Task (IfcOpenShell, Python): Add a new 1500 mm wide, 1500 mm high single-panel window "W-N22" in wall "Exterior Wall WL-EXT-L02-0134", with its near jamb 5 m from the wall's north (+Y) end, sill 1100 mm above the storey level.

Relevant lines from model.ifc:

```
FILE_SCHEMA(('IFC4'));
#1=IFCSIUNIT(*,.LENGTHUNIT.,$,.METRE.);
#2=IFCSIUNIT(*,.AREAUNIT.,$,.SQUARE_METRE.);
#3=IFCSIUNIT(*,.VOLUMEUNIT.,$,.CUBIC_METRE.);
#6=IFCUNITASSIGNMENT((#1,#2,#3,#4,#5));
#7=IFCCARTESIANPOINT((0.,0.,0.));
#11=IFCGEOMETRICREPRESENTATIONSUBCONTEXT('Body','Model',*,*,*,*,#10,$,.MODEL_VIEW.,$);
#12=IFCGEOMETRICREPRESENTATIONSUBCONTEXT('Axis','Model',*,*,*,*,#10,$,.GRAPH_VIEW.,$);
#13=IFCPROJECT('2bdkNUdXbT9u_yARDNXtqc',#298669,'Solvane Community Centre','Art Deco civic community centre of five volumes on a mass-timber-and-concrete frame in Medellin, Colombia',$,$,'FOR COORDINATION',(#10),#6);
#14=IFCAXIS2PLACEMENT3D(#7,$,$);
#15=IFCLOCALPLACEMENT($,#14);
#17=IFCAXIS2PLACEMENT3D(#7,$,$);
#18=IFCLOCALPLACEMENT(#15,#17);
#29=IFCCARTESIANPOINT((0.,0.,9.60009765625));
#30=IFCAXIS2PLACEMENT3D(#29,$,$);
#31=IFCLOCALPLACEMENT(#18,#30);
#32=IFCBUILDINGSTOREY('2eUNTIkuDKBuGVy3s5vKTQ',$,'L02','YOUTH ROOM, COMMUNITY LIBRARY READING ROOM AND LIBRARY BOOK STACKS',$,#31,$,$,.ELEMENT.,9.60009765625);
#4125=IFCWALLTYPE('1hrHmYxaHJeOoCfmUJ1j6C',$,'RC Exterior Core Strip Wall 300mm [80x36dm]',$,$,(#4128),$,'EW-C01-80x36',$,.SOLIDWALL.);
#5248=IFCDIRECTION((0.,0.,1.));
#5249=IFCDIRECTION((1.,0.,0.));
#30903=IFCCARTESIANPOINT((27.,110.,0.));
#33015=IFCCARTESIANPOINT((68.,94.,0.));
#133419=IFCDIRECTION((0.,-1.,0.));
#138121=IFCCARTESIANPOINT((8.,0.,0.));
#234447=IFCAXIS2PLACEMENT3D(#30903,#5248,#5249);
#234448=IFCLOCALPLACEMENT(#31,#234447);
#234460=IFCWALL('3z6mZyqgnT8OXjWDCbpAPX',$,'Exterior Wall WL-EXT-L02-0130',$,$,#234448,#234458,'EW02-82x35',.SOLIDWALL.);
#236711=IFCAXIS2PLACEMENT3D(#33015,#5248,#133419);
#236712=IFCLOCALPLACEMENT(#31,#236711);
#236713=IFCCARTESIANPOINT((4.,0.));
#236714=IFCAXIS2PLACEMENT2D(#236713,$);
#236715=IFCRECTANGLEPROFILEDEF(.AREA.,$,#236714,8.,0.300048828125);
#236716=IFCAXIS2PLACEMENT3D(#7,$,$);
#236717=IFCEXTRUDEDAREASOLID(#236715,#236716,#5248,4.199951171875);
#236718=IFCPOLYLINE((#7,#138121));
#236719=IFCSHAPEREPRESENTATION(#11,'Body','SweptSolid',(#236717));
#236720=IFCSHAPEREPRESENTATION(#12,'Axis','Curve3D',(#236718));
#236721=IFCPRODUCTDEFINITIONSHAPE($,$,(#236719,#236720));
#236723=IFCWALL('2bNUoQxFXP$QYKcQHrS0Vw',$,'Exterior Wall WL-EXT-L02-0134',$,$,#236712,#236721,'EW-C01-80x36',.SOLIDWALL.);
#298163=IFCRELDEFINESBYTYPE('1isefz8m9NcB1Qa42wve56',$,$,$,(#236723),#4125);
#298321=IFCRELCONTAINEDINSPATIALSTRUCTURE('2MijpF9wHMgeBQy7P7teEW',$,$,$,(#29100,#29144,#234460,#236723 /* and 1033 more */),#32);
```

```python
import numpy as np
import ifcopenshell
import ifcopenshell.api.feature
import ifcopenshell.api.geometry
import ifcopenshell.api.root
import ifcopenshell.api.spatial
import ifcopenshell.geom
import ifcopenshell.util.element
import ifcopenshell.util.placement
import ifcopenshell.util.representation
import ifcopenshell.util.shape
import ifcopenshell.util.unit

model = ifcopenshell.open("model.ifc")
unit_scale = ifcopenshell.util.unit.calculate_unit_scale(model)
settings = ifcopenshell.geom.settings()


def volume(element):
    """Net volume in cubic metres, openings subtracted."""
    shape = ifcopenshell.geom.create_shape(settings, element)
    return ifcopenshell.util.shape.get_volume(shape.geometry)


wall = model.by_guid("2bNUoQxFXP$QYKcQHrS0Vw")
storey = ifcopenshell.util.element.get_container(wall, ifc_class="IfcBuildingStorey")
context = ifcopenshell.util.representation.get_context(model, "Model", "Body", "MODEL_VIEW")
before = volume(wall)

width, height, from_end, sill = 1.5, 1.5, 5, 1.1  # metres

# The wall runs along its own X axis, and the end named is its -X end.
wall_shape = ifcopenshell.geom.create_shape(settings, wall)
x, y, z = ifcopenshell.util.shape.get_vertices(wall_shape.geometry).T
start = x.min() + from_end
face, thickness = float(y.min()), float(y.max() - y.min())
wall_matrix = ifcopenshell.util.placement.get_local_placement(wall.ObjectPlacement)
level = ifcopenshell.util.placement.get_local_placement(storey.ObjectPlacement)[2, 3]


def in_wall(x, y):
    """Placement at x, y metres in the wall's axes, at sill height."""
    matrix = wall_matrix.copy()
    matrix[:, 3] = wall_matrix @ np.array([x / unit_scale, y / unit_scale, 0.0, 1.0])
    matrix[2, 3] = level + sill / unit_scale
    return matrix


# Opening: a box that overshoots both wall faces by 50 mm.
opening = ifcopenshell.api.root.create_entity(model, ifc_class="IfcOpeningElement", predefined_type="OPENING")
box = ifcopenshell.api.geometry.add_wall_representation(
    model, context=context, length=width, height=height, thickness=thickness + 0.1
)
ifcopenshell.api.geometry.assign_representation(model, product=opening, representation=box)
ifcopenshell.api.geometry.edit_object_placement(model, product=opening, matrix=in_wall(start, face - 0.05), is_si=False)
ifcopenshell.api.feature.add_feature(model, feature=opening, element=wall)

window = ifcopenshell.api.root.create_entity(model, ifc_class="IfcWindow", name="W-N22", predefined_type="WINDOW")
window.OverallWidth, window.OverallHeight = width / unit_scale, height / unit_scale
window.PartitioningType = "SINGLE_PANEL"
body = ifcopenshell.api.geometry.add_window_representation(
    model,
    context=context,
    overall_width=window.OverallWidth,
    overall_height=window.OverallHeight,
    partition_type="SINGLE_PANEL",
)
ifcopenshell.api.geometry.assign_representation(model, product=window, representation=body)
ifcopenshell.api.spatial.assign_container(model, products=[window], relating_structure=storey)
ifcopenshell.api.feature.add_filling(model, opening=opening, element=window)

# Centre the window in the wall's thickness.
ifcopenshell.api.geometry.edit_object_placement(model, product=window, matrix=in_wall(start, face), is_si=False)
window_shape = ifcopenshell.geom.create_shape(settings, window)
depth = ifcopenshell.util.shape.get_vertices(window_shape.geometry)[:, 1]
offset = face + thickness / 2 - (depth.min() + depth.max()) / 2
ifcopenshell.api.geometry.edit_object_placement(model, product=window, matrix=in_wall(start, offset), is_si=False)

after = volume(wall)

print(f"wall volume {before:.3f} -> {after:.3f} m3")

model.write("model_v2.ifc")
```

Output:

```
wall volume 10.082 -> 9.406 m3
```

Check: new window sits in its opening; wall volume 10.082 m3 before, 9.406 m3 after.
